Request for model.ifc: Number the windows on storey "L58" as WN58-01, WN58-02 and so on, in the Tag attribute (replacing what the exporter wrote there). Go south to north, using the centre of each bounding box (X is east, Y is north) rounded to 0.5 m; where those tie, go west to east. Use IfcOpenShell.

First a look at what the model holds.

```python
import ifcopenshell
import ifcopenshell.util.element
import ifcopenshell.util.placement

model = ifcopenshell.open("model.ifc")
print(model.schema)
storey = next(s for s in model.by_type("IfcBuildingStorey") if s.Name == "L58")
windows = [e for e in ifcopenshell.util.element.get_decomposition(storey) if e.is_a("IfcWindow")]
for e in sorted(windows, key=lambda e: e.id()):
    origin = ifcopenshell.util.placement.get_local_placement(e.ObjectPlacement)[:3, 3]
    print(e.id(), e.Tag, e.Name, origin.round(2) + 0.0, sep=" | ")
```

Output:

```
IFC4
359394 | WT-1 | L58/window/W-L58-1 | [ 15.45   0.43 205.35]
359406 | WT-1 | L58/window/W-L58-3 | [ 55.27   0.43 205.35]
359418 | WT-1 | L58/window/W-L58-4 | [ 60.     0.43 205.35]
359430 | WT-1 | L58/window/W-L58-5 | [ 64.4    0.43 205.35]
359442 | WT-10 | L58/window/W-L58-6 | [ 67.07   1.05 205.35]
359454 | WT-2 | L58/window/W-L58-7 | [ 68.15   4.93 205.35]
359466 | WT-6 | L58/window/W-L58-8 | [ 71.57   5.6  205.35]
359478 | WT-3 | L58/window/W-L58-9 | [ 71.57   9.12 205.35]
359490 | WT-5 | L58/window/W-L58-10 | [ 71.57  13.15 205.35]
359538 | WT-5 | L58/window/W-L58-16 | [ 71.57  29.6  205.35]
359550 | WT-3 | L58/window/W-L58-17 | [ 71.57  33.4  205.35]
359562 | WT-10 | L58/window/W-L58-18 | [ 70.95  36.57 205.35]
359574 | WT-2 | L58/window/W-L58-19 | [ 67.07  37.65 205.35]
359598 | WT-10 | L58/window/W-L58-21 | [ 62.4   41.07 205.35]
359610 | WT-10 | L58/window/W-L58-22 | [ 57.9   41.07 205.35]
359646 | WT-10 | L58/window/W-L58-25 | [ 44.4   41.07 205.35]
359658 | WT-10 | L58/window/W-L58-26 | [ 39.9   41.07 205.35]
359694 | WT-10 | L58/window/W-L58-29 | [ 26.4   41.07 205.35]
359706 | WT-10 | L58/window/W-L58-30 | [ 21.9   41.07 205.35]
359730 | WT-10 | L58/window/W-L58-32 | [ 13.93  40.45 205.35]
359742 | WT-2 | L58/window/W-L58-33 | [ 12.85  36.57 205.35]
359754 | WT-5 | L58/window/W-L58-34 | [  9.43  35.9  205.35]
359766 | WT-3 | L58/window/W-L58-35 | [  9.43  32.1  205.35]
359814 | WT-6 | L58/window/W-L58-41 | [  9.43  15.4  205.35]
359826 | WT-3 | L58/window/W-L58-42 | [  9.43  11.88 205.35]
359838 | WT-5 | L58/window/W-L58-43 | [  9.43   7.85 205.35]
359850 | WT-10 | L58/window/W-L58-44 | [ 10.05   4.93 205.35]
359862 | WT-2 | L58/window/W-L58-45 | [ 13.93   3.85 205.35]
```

```python
import ifcopenshell
import ifcopenshell.geom
import ifcopenshell.util.element
import ifcopenshell.util.shape

model = ifcopenshell.open("model.ifc")
settings = ifcopenshell.geom.settings()
settings.set("use-world-coords", True)


def centre(element):
    shape = ifcopenshell.geom.create_shape(settings, element)
    return ifcopenshell.util.shape.get_bbox_centroid(shape.geometry)


storey = next(s for s in model.by_type("IfcBuildingStorey") if s.Name == "L58")
windows = [e for e in ifcopenshell.util.element.get_decomposition(storey) if e.is_a("IfcWindow")]

# Insertion points can sit at a corner or the storey origin, so sort by the geometry (in metres).
centres = {e: centre(e) for e in windows}
windows.sort(key=lambda e: (round(centres[e][1] / 0.5), centres[e][0]))

for i, e in enumerate(windows, start=1):
    number = f"WN58-{i:02d}"
    e.Tag = number
    print(e.id(), number)

model.write("model_updated.ifc")
```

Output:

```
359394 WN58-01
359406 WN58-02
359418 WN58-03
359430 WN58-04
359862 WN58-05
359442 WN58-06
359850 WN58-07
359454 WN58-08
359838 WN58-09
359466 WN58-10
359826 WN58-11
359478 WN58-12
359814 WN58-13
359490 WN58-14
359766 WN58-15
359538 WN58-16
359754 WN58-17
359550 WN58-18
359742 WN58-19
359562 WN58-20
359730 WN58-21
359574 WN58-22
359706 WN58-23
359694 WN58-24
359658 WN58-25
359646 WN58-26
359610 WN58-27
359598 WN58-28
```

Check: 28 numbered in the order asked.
